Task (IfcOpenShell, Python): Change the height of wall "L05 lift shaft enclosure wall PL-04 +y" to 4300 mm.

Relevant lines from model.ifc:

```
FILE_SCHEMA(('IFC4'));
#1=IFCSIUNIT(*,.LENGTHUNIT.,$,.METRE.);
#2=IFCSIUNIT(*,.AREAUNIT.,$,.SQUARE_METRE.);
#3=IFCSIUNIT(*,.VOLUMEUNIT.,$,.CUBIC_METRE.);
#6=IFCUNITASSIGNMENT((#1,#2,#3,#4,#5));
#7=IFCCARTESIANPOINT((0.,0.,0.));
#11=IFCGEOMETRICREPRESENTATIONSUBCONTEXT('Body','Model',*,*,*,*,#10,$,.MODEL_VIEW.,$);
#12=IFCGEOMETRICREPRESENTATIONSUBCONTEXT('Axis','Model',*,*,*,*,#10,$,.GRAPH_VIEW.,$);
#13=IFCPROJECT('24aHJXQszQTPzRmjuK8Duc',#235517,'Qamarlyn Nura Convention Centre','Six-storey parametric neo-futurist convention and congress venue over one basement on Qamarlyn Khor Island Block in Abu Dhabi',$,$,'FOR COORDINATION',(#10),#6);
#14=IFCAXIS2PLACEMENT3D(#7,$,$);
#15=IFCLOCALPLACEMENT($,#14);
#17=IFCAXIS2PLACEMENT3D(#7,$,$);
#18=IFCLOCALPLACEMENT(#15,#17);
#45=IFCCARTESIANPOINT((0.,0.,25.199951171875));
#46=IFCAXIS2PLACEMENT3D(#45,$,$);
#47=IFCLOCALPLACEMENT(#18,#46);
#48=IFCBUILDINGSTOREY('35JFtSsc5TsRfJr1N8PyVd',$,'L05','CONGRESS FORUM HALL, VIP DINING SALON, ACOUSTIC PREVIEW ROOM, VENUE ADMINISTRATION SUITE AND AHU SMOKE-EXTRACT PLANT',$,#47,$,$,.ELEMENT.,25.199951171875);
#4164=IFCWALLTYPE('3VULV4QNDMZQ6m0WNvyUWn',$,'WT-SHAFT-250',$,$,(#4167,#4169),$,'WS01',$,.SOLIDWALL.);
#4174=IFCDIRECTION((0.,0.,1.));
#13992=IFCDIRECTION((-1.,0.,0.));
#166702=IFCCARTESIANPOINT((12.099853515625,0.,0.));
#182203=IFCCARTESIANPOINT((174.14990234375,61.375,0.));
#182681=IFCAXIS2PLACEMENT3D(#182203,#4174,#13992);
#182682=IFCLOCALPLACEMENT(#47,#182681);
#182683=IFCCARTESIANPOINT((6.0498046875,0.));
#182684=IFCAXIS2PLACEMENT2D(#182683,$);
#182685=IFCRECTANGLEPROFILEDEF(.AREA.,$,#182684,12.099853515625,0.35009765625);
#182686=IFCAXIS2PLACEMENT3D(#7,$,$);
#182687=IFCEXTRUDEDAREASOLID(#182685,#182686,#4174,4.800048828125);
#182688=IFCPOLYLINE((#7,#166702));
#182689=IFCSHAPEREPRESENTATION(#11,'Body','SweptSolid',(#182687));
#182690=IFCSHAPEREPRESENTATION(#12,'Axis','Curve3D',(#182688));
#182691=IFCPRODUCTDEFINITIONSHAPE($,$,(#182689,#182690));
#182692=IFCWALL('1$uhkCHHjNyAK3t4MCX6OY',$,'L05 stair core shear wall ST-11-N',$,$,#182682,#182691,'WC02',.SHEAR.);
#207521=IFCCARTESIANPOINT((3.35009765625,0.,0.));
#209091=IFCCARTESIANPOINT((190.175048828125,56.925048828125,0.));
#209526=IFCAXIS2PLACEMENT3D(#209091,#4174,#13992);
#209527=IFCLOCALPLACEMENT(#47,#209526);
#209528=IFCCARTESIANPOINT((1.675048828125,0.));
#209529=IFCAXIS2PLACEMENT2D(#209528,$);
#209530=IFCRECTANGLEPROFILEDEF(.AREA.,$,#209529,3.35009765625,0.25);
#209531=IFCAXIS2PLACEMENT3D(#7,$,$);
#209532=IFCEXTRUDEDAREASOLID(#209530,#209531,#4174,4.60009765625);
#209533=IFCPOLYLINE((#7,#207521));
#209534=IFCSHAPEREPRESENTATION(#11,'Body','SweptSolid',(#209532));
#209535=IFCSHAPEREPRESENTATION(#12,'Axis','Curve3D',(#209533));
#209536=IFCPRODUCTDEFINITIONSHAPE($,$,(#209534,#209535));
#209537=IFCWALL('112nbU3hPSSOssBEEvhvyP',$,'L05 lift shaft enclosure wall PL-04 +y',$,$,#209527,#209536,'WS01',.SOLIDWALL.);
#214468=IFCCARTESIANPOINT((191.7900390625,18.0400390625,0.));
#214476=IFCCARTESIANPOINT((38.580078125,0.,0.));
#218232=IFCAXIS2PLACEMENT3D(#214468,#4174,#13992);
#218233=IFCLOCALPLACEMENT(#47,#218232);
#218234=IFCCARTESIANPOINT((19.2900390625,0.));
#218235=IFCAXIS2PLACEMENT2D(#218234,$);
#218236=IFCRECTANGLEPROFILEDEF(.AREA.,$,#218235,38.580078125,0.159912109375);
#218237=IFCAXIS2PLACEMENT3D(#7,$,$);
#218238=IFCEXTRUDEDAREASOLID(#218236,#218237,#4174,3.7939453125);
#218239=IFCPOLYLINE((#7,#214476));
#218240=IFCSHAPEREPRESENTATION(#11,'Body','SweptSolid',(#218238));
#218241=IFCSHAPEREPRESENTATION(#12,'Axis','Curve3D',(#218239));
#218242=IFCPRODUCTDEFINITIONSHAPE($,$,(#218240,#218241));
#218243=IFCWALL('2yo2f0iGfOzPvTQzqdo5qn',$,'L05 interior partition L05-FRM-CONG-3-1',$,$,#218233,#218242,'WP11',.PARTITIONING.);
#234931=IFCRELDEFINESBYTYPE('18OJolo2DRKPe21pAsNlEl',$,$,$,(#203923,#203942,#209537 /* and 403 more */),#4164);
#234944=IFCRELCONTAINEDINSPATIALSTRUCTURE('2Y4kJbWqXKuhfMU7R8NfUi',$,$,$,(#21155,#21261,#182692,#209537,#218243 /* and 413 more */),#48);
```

```python
import ifcopenshell
import ifcopenshell.geom
import ifcopenshell.util.representation
import ifcopenshell.util.shape
import ifcopenshell.util.unit

model = ifcopenshell.open("model.ifc")
unit_scale = ifcopenshell.util.unit.calculate_unit_scale(model)
settings = ifcopenshell.geom.settings()


def volume(element):
    """Net volume in cubic metres, openings subtracted."""
    shape = ifcopenshell.geom.create_shape(settings, element)
    return ifcopenshell.util.shape.get_volume(shape.geometry)


wall = model.by_guid("112nbU3hPSSOssBEEvhvyP")
before = volume(wall)

body = ifcopenshell.util.representation.get_representation(wall, "Model", "Body")
solid = body.Items[0]
old_height = solid.Depth
solid.Depth = 4.3 / unit_scale
after = volume(wall)

print(f"height {old_height:g} -> {solid.Depth:g}, volume {before:.3f} -> {after:.3f} m3")

model.write("model_v2.ifc")
```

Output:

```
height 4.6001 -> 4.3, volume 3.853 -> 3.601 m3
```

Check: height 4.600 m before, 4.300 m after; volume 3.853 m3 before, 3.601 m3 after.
